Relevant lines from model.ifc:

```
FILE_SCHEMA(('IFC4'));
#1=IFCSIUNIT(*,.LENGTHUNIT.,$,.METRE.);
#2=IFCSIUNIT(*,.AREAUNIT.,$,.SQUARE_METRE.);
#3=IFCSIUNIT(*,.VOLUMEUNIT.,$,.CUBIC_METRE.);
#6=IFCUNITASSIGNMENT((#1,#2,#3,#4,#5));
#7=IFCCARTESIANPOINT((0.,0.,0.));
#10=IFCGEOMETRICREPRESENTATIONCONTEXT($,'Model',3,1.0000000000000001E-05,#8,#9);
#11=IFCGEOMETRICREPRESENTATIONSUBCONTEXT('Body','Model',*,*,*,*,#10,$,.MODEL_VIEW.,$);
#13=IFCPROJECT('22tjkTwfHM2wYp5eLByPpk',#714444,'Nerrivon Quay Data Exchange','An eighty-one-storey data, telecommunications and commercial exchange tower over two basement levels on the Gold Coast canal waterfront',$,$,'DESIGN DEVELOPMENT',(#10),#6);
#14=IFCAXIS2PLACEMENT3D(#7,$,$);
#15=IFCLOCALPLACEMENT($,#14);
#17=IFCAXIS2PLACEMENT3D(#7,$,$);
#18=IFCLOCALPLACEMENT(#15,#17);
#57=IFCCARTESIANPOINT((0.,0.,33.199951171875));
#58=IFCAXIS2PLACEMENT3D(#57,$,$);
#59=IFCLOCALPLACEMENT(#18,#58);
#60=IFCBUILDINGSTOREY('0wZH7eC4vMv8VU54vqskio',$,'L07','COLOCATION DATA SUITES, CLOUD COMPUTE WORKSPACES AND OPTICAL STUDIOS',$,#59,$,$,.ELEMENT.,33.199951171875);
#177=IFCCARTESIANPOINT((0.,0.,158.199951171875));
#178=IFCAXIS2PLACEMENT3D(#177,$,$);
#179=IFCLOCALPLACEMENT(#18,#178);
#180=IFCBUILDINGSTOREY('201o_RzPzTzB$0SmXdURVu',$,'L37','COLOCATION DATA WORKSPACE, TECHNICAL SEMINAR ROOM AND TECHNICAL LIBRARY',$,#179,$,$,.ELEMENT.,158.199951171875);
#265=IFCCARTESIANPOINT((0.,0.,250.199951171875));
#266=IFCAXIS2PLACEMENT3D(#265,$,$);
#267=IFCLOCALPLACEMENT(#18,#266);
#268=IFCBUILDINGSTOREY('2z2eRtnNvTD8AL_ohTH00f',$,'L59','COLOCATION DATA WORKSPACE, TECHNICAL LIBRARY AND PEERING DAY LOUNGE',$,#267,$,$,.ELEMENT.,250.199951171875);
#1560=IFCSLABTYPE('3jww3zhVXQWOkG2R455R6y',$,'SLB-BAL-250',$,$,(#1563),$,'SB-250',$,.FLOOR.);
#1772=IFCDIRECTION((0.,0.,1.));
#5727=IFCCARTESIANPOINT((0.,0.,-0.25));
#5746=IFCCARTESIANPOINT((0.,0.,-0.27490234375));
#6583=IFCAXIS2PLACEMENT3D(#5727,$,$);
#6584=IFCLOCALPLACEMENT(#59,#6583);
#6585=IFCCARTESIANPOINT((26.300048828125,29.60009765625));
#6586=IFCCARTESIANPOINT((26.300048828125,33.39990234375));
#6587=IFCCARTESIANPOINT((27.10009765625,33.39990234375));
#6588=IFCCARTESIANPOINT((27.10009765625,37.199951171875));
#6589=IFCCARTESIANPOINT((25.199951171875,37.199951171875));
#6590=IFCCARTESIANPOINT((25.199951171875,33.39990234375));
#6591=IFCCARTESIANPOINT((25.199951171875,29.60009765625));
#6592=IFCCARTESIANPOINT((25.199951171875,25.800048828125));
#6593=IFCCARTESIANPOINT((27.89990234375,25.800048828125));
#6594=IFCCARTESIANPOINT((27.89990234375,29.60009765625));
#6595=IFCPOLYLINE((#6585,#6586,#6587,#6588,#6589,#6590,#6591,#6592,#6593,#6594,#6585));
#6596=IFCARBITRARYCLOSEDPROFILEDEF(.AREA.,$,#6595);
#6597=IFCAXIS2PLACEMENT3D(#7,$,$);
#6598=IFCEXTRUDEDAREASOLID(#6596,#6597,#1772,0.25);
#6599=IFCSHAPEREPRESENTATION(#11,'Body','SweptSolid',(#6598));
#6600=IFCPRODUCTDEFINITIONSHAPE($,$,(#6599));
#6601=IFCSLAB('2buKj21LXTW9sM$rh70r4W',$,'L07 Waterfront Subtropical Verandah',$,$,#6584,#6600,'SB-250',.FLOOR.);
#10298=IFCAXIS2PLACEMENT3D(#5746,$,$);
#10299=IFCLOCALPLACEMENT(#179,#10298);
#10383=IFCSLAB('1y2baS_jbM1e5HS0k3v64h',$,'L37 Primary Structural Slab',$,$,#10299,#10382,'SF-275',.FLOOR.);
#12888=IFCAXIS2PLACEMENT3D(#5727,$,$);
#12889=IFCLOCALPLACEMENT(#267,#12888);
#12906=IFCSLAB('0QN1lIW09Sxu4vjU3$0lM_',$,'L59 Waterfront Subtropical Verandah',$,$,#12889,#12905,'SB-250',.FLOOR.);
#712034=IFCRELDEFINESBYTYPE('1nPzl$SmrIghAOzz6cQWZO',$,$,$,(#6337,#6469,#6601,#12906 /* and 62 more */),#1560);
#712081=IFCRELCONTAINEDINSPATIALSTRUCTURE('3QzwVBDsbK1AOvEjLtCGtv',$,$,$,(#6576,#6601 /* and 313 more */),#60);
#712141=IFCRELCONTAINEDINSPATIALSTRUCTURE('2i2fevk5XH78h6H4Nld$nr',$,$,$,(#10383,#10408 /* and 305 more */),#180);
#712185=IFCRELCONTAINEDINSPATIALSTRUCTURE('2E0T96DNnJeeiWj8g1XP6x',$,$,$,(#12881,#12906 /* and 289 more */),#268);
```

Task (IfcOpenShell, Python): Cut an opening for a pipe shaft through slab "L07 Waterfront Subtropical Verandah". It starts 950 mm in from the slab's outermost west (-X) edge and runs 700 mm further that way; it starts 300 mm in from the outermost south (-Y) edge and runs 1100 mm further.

```python
import numpy as np
import ifcopenshell
import ifcopenshell.api.feature
import ifcopenshell.api.geometry
import ifcopenshell.api.root
import ifcopenshell.geom
import ifcopenshell.util.placement
import ifcopenshell.util.representation
import ifcopenshell.util.shape
import ifcopenshell.util.unit

model = ifcopenshell.open("model.ifc")
unit_scale = ifcopenshell.util.unit.calculate_unit_scale(model)
settings = ifcopenshell.geom.settings()


def volume(element):
    """Net volume in cubic metres, openings subtracted."""
    shape = ifcopenshell.geom.create_shape(settings, element)
    return ifcopenshell.util.shape.get_volume(shape.geometry)


slab = model.by_guid("2buKj21LXTW9sM$rh70r4W")
before = volume(slab)

# Extent in the slab's own axes, in metres. The edges named are its -X and -Y sides.
slab_shape = ifcopenshell.geom.create_shape(settings, slab)
vertices = ifcopenshell.util.shape.get_vertices(slab_shape.geometry)
x_min, y_min, bottom = vertices.min(axis=0)
top = vertices[:, 2].max()

opening = ifcopenshell.api.root.create_entity(model, ifc_class="IfcOpeningElement", name="Pipe shaft opening", predefined_type="OPENING")
context = ifcopenshell.util.representation.get_context(model, "Model", "Body", "MODEL_VIEW")
width, depth = 0.7, 1.1
outline = [(0.0, 0.0), (width, 0.0), (width, depth), (0.0, depth), (0.0, 0.0)]
# Overshoot both faces by 50 mm so the cut is clean.
shape = ifcopenshell.api.geometry.add_slab_representation(
    model, context=context, depth=top - bottom + 0.1, polyline=outline
)
ifcopenshell.api.geometry.assign_representation(model, product=opening, representation=shape)

matrix = ifcopenshell.util.placement.get_local_placement(slab.ObjectPlacement)
matrix[:, 3] = matrix @ np.append(np.array([x_min + 0.95, y_min + 0.3, bottom - 0.05]) / unit_scale, 1.0)
ifcopenshell.api.geometry.edit_object_placement(model, product=opening, matrix=matrix, is_si=False)
ifcopenshell.api.feature.add_feature(model, feature=opening, element=slab)

after = volume(slab)

print(f"slab volume {before:.3f} -> {after:.3f} m3")

model.write("model_edited.ifc")
```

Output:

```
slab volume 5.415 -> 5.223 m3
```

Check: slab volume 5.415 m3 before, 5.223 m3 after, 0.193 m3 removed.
